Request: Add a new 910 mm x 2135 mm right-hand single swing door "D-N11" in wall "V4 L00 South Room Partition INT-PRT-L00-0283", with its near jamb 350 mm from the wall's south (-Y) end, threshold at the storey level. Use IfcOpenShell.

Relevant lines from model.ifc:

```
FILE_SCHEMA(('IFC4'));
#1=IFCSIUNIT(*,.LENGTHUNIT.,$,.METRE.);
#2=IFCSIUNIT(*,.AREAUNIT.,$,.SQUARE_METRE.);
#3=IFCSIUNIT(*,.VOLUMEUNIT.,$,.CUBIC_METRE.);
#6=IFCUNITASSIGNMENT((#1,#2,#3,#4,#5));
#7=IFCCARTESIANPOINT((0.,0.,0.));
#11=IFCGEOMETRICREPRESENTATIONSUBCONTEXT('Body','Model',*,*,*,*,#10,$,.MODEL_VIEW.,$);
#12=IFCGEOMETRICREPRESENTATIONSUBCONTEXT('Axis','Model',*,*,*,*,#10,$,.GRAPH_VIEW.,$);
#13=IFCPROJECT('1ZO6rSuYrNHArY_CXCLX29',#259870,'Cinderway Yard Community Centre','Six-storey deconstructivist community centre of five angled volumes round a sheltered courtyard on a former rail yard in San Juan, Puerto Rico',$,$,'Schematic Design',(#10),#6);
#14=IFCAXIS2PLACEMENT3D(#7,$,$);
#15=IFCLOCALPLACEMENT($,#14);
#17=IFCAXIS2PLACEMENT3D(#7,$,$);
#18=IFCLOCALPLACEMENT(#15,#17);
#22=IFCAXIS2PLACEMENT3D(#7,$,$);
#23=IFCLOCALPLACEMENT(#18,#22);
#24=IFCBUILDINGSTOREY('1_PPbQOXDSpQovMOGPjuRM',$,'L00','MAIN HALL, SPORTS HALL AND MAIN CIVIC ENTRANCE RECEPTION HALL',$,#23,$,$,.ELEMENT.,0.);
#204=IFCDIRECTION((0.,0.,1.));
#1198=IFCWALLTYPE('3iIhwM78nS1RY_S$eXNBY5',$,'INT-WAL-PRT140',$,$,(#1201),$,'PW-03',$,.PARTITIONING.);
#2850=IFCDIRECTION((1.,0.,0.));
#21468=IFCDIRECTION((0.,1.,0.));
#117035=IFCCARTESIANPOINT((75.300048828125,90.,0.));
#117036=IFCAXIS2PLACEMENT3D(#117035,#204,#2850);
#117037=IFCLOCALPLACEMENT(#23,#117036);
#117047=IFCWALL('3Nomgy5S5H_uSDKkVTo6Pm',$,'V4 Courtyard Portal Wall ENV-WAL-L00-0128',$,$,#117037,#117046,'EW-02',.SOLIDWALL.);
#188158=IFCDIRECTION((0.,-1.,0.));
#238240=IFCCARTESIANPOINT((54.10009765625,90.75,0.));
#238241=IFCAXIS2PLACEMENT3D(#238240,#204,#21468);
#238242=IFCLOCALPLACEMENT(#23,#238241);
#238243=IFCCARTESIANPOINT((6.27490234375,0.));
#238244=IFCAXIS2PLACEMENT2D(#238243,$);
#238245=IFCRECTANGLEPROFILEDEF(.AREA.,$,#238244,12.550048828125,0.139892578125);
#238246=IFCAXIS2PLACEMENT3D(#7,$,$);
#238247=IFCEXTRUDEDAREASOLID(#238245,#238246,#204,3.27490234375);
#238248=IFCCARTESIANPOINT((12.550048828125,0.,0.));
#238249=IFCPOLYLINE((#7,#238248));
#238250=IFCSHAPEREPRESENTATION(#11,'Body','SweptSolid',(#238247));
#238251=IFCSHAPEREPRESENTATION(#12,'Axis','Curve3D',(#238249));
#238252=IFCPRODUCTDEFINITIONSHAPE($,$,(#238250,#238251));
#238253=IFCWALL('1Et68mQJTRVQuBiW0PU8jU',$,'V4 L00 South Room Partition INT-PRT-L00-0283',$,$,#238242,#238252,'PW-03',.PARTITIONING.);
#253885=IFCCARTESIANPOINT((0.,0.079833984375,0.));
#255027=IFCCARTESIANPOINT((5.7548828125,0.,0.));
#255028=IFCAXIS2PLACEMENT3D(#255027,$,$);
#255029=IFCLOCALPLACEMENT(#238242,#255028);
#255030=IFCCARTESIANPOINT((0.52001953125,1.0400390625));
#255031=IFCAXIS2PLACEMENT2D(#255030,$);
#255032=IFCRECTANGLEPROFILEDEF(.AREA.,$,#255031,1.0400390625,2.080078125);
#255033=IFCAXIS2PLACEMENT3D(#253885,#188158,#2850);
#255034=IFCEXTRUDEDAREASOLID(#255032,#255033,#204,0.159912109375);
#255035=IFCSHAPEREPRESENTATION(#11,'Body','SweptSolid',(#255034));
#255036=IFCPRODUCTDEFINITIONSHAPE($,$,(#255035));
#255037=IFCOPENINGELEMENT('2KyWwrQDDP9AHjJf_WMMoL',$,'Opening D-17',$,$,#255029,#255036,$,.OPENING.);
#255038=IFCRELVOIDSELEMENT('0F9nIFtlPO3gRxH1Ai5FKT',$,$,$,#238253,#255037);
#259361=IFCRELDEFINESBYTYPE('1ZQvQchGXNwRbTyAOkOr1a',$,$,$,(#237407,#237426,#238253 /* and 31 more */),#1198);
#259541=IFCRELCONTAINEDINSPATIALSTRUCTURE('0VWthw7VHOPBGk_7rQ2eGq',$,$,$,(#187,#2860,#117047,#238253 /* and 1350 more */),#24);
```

```python
import numpy as np
import ifcopenshell
import ifcopenshell.api.feature
import ifcopenshell.api.geometry
import ifcopenshell.api.root
import ifcopenshell.api.spatial
import ifcopenshell.geom
import ifcopenshell.util.element
import ifcopenshell.util.placement
import ifcopenshell.util.representation
import ifcopenshell.util.shape
import ifcopenshell.util.unit

model = ifcopenshell.open("model.ifc")
unit_scale = ifcopenshell.util.unit.calculate_unit_scale(model)
settings = ifcopenshell.geom.settings()


def volume(element):
    """Net volume in cubic metres, openings subtracted."""
    shape = ifcopenshell.geom.create_shape(settings, element)
    return ifcopenshell.util.shape.get_volume(shape.geometry)


wall = model.by_id(238253)
storey = ifcopenshell.util.element.get_container(wall, ifc_class="IfcBuildingStorey")
context = ifcopenshell.util.representation.get_context(model, "Model", "Body", "MODEL_VIEW")
before = volume(wall)

width, height, from_end, sill = 0.91, 2.135, 0.35, 0.0  # metres

# The wall runs along its own X axis, and the end named is its -X end.
wall_shape = ifcopenshell.geom.create_shape(settings, wall)
x, y, z = ifcopenshell.util.shape.get_vertices(wall_shape.geometry).T
start = x.min() + from_end
face, thickness = float(y.min()), float(y.max() - y.min())
wall_matrix = ifcopenshell.util.placement.get_local_placement(wall.ObjectPlacement)
level = ifcopenshell.util.placement.get_local_placement(storey.ObjectPlacement)[2, 3]


def in_wall(x, y):
    """Placement at x, y metres in the wall's axes, at sill height."""
    matrix = wall_matrix.copy()
    matrix[:, 3] = wall_matrix @ np.array([x / unit_scale, y / unit_scale, 0.0, 1.0])
    matrix[2, 3] = level + sill / unit_scale
    return matrix


# Opening: a box that overshoots both wall faces by 50 mm.
opening = ifcopenshell.api.root.create_entity(model, ifc_class="IfcOpeningElement", predefined_type="OPENING")
box = ifcopenshell.api.geometry.add_wall_representation(
    model, context=context, length=width, height=height, thickness=thickness + 0.1
)
ifcopenshell.api.geometry.assign_representation(model, product=opening, representation=box)
ifcopenshell.api.geometry.edit_object_placement(model, product=opening, matrix=in_wall(start, face - 0.05), is_si=False)
ifcopenshell.api.feature.add_feature(model, feature=opening, element=wall)

door = ifcopenshell.api.root.create_entity(model, ifc_class="IfcDoor", name="D-N11", predefined_type="DOOR")
door.OverallWidth, door.OverallHeight = width / unit_scale, height / unit_scale
door.OperationType = "SINGLE_SWING_RIGHT"
body = ifcopenshell.api.geometry.add_door_representation(
    model,
    context=context,
    overall_width=door.OverallWidth,
    overall_height=door.OverallHeight,
    operation_type="SINGLE_SWING_RIGHT",
    lining_properties={"LiningDepth": thickness / unit_scale, "ThresholdDepth": thickness / unit_scale},
)
ifcopenshell.api.geometry.assign_representation(model, product=door, representation=body)
ifcopenshell.api.spatial.assign_container(model, products=[door], relating_structure=storey)
ifcopenshell.api.feature.add_filling(model, opening=opening, element=door)

# The lining spans the wall, so the door starts at the wall face.
ifcopenshell.api.geometry.edit_object_placement(model, product=door, matrix=in_wall(start, face), is_si=False)

after = volume(wall)

print(f"wall volume {before:.3f} -> {after:.3f} m3")

model.write("model_v2.ifc")
```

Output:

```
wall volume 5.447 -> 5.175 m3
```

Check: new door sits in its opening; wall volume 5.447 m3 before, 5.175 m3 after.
